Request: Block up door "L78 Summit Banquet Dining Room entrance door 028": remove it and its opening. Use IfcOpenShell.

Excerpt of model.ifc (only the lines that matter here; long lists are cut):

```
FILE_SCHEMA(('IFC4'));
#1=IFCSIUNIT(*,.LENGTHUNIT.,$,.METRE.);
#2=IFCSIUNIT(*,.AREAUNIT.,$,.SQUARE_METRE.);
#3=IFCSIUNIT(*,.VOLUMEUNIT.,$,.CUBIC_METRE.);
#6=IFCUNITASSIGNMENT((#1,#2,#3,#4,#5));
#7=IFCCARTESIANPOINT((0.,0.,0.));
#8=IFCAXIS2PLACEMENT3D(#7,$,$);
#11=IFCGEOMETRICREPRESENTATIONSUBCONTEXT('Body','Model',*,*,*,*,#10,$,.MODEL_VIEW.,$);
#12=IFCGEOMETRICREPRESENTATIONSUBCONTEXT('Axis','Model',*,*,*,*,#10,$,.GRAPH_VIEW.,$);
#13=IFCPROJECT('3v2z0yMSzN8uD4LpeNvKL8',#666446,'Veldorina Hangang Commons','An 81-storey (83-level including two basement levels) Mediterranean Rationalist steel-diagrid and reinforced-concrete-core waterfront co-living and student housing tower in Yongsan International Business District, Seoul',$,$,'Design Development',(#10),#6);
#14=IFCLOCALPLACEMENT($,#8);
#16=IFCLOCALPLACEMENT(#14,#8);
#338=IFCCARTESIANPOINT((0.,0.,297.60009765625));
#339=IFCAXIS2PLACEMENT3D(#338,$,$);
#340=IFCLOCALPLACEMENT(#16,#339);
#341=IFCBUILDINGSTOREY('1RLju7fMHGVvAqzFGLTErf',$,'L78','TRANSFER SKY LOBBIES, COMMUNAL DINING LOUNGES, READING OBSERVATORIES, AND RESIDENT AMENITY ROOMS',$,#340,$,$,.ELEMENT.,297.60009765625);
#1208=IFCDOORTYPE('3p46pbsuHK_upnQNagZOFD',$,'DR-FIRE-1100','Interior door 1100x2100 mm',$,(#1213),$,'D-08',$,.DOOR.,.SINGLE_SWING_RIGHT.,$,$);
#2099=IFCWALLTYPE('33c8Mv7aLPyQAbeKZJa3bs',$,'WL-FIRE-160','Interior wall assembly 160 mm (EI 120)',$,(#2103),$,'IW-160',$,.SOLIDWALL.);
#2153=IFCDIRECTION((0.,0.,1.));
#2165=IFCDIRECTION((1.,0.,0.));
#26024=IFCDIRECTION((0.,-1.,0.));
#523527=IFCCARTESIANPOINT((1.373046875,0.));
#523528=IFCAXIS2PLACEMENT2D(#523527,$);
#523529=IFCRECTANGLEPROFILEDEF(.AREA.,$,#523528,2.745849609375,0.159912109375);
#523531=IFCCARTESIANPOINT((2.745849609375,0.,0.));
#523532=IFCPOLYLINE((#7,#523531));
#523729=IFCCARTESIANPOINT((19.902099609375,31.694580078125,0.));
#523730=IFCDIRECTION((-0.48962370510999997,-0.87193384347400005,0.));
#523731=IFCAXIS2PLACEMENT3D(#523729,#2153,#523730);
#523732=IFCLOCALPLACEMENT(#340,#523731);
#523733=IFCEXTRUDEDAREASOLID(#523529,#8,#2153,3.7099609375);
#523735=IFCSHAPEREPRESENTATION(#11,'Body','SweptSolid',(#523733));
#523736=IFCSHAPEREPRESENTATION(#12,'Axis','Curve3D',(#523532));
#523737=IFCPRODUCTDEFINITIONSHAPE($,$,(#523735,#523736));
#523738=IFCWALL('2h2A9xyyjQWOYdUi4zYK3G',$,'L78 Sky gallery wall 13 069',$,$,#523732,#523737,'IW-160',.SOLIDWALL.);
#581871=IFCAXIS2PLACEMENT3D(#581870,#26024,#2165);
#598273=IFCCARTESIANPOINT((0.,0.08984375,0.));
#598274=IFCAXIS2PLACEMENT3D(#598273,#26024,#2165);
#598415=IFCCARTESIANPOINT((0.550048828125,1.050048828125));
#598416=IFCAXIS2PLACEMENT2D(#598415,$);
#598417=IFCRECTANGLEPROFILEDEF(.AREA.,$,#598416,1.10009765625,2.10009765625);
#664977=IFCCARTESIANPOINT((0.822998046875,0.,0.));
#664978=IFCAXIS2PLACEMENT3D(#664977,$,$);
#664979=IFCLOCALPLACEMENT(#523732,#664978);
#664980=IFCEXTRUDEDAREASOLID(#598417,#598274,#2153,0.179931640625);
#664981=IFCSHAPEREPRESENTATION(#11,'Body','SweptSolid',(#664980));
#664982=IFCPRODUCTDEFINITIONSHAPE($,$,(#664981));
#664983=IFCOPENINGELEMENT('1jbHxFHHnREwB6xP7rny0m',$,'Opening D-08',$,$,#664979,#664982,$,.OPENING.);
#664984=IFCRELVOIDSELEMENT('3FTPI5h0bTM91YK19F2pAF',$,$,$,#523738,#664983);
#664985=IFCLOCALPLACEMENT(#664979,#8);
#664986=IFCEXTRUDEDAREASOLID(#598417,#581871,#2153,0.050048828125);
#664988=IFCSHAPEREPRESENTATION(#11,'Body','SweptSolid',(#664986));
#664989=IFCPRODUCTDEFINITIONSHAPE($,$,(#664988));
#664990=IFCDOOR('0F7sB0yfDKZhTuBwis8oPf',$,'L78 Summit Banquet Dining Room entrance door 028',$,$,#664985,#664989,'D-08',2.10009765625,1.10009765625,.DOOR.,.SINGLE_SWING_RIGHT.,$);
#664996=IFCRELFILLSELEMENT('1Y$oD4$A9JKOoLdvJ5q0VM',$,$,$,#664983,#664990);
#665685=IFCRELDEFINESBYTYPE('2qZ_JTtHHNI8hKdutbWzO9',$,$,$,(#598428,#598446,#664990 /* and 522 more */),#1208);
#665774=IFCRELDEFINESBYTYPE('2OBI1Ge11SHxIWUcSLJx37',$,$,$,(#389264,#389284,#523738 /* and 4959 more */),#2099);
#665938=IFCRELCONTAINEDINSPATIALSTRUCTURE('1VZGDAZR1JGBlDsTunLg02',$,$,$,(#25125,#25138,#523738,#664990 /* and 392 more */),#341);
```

```python
import ifcopenshell
import ifcopenshell.api.feature
import ifcopenshell.api.root
import ifcopenshell.geom
import ifcopenshell.util.shape

model = ifcopenshell.open("model.ifc")
settings = ifcopenshell.geom.settings()


def volume(element):
    """Net volume in cubic metres, openings subtracted."""
    shape = ifcopenshell.geom.create_shape(settings, element)
    return ifcopenshell.util.shape.get_volume(shape.geometry)


door = model.by_guid("0F7sB0yfDKZhTuBwis8oPf")
opening = door.FillsVoids[0].RelatingOpeningElement
wall = opening.VoidsElements[0].RelatingBuildingElement
before = volume(wall)

ifcopenshell.api.root.remove_product(model, product=door)
ifcopenshell.api.feature.remove_feature(model, feature=opening)

after = volume(wall)

print(f"wall volume {before:.3f} -> {after:.3f} m3")

model.write("model_rev.ifc")
```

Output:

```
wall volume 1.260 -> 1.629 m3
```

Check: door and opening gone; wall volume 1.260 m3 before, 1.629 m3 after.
